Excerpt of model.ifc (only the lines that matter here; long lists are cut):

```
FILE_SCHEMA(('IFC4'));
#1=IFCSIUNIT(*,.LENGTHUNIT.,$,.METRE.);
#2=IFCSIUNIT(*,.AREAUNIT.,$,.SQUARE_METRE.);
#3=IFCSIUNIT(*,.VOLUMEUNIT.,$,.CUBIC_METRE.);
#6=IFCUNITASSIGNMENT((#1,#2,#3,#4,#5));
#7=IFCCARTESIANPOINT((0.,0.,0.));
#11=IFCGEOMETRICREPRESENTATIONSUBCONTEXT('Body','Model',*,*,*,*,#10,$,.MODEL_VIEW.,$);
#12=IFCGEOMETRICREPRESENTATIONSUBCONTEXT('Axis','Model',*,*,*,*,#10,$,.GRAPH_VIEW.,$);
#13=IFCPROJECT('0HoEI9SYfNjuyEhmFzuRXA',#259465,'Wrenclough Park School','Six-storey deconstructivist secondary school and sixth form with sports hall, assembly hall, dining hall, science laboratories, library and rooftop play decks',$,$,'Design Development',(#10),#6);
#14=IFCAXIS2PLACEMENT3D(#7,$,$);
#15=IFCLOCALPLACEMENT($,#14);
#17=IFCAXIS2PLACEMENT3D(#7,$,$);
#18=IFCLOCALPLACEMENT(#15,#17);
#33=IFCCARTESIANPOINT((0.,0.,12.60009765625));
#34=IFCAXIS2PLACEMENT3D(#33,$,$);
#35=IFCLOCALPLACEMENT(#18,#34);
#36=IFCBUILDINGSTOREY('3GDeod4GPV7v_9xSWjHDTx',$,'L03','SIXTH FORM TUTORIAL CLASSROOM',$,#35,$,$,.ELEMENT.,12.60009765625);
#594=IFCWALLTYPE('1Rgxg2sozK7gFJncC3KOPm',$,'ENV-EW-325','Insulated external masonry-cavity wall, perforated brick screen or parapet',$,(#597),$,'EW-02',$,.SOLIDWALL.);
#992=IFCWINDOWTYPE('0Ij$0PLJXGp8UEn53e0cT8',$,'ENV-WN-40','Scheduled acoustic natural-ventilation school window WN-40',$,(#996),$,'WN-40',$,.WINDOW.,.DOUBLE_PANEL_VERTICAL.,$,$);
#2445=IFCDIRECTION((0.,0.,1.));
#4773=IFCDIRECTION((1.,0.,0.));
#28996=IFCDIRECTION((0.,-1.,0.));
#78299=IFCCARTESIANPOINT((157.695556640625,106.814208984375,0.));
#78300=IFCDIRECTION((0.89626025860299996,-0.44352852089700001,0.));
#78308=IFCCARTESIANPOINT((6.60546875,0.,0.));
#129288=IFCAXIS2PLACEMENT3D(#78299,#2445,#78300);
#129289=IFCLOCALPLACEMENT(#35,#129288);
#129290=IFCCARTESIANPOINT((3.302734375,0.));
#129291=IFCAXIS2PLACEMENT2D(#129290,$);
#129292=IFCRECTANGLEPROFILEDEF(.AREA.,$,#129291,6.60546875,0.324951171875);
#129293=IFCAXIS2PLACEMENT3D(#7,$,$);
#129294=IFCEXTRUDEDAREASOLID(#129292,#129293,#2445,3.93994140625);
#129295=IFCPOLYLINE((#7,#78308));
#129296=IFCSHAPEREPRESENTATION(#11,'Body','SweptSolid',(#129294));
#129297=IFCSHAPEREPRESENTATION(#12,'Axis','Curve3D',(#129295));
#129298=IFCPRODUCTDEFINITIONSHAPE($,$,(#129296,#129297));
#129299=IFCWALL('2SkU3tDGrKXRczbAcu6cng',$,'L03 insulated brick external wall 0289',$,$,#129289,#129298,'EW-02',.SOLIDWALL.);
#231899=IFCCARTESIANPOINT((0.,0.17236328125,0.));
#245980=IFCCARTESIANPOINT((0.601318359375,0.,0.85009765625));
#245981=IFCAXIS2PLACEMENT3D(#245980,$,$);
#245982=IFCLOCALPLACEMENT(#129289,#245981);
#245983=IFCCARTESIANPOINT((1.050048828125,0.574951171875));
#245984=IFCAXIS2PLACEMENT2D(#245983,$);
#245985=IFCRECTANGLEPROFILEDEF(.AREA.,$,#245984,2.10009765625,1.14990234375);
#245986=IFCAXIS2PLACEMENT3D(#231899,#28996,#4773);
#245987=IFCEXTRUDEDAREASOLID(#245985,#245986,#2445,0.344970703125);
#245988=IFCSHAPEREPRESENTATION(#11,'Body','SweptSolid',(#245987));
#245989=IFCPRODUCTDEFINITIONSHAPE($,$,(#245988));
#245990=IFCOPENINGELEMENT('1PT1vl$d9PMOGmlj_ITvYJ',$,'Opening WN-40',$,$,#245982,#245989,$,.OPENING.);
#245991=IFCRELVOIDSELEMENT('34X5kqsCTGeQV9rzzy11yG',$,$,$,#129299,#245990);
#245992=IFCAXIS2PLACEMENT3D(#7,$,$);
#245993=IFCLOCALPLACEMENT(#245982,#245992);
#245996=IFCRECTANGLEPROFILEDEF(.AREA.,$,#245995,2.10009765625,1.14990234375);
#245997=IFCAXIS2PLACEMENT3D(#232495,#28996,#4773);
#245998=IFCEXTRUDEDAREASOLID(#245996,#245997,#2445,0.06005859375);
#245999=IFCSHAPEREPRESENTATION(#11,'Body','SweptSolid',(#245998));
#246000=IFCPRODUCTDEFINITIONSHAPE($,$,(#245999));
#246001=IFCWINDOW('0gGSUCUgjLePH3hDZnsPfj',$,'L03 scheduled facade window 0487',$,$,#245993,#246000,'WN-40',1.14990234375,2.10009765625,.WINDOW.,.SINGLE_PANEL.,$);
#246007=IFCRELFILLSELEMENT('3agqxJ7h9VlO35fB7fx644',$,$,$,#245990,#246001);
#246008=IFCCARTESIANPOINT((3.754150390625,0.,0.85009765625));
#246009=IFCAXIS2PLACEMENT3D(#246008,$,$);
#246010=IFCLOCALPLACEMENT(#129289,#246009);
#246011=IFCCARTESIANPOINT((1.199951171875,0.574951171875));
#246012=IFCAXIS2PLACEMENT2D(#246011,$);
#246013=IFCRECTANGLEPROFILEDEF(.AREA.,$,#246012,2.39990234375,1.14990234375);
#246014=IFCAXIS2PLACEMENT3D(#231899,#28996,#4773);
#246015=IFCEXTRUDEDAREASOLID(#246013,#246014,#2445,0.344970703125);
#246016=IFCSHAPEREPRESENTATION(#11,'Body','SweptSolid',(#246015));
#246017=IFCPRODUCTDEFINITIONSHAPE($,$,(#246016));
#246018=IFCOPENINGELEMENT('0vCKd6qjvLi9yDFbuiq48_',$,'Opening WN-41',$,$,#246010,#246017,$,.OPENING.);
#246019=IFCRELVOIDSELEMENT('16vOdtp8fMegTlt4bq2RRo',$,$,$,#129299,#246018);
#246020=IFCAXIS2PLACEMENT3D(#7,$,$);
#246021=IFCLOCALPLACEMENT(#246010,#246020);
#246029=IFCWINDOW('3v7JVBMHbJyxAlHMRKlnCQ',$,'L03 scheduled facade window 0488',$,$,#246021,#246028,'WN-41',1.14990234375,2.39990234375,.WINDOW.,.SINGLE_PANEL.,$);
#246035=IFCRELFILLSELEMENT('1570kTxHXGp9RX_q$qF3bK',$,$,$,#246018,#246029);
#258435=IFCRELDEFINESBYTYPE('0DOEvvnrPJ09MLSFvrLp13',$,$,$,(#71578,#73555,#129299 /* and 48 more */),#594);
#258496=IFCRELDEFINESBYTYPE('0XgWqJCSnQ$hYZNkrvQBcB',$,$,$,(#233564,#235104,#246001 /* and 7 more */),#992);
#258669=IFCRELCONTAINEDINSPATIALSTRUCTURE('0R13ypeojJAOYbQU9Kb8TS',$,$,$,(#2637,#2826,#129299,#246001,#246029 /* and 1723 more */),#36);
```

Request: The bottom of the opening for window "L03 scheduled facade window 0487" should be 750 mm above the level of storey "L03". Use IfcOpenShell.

```python
import numpy as np
import ifcopenshell
import ifcopenshell.api.geometry
import ifcopenshell.geom
import ifcopenshell.util.element
import ifcopenshell.util.placement
import ifcopenshell.util.shape
import ifcopenshell.util.unit

model = ifcopenshell.open("model.ifc")
unit_scale = ifcopenshell.util.unit.calculate_unit_scale(model)

window = model.by_guid("0gGSUCUgjLePH3hDZnsPfj")
opening = window.FillsVoids[0].RelatingOpeningElement
storey = ifcopenshell.util.element.get_container(window, ifc_class="IfcBuildingStorey")
level = ifcopenshell.util.placement.get_local_placement(storey.ObjectPlacement)[2, 3]

# The opening's origin need not be at the sill, so measure its lowest point.
shape = ifcopenshell.geom.create_shape(ifcopenshell.geom.settings(), opening)
bottom = ifcopenshell.util.shape.get_shape_bottom_elevation(shape, shape.geometry) / unit_scale
dz = level + 0.75 - bottom

shift = np.array([0.0, 0.0, dz])
# The window is placed relative to its opening, so it follows when the opening moves.
matrix = ifcopenshell.util.placement.get_local_placement(opening.ObjectPlacement)
matrix[:3, 3] += shift
ifcopenshell.api.geometry.edit_object_placement(
    model, product=opening, matrix=matrix, is_si=False, should_transform_children=True
)

print(f"moved by {dz * unit_scale:+.3f} m")

model.write("model_v2.ifc")
```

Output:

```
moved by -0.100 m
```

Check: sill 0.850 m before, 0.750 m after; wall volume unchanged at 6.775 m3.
